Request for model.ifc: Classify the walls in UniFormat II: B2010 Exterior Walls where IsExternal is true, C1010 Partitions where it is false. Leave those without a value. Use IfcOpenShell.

First a look at what the model holds.

```python
import ifcopenshell
import ifcopenshell.util.element

model = ifcopenshell.open("model.ifc")
print(model.schema)
print("classifications:", [c.Name for c in model.by_type("IfcClassification")])
values = [ifcopenshell.util.element.get_pset(e, "Pset_WallCommon", "IsExternal") for e in model.by_type("IfcWall")]
for value in (True, False, None):
    print("IsExternal", value, values.count(value))
```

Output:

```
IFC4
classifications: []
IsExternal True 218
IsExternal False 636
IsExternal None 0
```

```python
import ifcopenshell
import ifcopenshell.api.classification
import ifcopenshell.util.element

model = ifcopenshell.open("model.ifc")

system = ifcopenshell.api.classification.add_classification(model, classification="UniFormat II")

walls = model.by_type("IfcWall")
external = {e: ifcopenshell.util.element.get_pset(e, "Pset_WallCommon", "IsExternal") for e in walls}
for flag, code, name in ((True, "B2010", "Exterior Walls"), (False, "C1010", "Partitions")):
    products = [e for e in walls if external[e] is flag]
    ifcopenshell.api.classification.add_reference(
        model, products=products, classification=system, identification=code, name=name
    )
    print(code, len(products))

model.write("model_updated.ifc")
```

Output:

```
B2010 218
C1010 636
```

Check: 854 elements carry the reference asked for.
